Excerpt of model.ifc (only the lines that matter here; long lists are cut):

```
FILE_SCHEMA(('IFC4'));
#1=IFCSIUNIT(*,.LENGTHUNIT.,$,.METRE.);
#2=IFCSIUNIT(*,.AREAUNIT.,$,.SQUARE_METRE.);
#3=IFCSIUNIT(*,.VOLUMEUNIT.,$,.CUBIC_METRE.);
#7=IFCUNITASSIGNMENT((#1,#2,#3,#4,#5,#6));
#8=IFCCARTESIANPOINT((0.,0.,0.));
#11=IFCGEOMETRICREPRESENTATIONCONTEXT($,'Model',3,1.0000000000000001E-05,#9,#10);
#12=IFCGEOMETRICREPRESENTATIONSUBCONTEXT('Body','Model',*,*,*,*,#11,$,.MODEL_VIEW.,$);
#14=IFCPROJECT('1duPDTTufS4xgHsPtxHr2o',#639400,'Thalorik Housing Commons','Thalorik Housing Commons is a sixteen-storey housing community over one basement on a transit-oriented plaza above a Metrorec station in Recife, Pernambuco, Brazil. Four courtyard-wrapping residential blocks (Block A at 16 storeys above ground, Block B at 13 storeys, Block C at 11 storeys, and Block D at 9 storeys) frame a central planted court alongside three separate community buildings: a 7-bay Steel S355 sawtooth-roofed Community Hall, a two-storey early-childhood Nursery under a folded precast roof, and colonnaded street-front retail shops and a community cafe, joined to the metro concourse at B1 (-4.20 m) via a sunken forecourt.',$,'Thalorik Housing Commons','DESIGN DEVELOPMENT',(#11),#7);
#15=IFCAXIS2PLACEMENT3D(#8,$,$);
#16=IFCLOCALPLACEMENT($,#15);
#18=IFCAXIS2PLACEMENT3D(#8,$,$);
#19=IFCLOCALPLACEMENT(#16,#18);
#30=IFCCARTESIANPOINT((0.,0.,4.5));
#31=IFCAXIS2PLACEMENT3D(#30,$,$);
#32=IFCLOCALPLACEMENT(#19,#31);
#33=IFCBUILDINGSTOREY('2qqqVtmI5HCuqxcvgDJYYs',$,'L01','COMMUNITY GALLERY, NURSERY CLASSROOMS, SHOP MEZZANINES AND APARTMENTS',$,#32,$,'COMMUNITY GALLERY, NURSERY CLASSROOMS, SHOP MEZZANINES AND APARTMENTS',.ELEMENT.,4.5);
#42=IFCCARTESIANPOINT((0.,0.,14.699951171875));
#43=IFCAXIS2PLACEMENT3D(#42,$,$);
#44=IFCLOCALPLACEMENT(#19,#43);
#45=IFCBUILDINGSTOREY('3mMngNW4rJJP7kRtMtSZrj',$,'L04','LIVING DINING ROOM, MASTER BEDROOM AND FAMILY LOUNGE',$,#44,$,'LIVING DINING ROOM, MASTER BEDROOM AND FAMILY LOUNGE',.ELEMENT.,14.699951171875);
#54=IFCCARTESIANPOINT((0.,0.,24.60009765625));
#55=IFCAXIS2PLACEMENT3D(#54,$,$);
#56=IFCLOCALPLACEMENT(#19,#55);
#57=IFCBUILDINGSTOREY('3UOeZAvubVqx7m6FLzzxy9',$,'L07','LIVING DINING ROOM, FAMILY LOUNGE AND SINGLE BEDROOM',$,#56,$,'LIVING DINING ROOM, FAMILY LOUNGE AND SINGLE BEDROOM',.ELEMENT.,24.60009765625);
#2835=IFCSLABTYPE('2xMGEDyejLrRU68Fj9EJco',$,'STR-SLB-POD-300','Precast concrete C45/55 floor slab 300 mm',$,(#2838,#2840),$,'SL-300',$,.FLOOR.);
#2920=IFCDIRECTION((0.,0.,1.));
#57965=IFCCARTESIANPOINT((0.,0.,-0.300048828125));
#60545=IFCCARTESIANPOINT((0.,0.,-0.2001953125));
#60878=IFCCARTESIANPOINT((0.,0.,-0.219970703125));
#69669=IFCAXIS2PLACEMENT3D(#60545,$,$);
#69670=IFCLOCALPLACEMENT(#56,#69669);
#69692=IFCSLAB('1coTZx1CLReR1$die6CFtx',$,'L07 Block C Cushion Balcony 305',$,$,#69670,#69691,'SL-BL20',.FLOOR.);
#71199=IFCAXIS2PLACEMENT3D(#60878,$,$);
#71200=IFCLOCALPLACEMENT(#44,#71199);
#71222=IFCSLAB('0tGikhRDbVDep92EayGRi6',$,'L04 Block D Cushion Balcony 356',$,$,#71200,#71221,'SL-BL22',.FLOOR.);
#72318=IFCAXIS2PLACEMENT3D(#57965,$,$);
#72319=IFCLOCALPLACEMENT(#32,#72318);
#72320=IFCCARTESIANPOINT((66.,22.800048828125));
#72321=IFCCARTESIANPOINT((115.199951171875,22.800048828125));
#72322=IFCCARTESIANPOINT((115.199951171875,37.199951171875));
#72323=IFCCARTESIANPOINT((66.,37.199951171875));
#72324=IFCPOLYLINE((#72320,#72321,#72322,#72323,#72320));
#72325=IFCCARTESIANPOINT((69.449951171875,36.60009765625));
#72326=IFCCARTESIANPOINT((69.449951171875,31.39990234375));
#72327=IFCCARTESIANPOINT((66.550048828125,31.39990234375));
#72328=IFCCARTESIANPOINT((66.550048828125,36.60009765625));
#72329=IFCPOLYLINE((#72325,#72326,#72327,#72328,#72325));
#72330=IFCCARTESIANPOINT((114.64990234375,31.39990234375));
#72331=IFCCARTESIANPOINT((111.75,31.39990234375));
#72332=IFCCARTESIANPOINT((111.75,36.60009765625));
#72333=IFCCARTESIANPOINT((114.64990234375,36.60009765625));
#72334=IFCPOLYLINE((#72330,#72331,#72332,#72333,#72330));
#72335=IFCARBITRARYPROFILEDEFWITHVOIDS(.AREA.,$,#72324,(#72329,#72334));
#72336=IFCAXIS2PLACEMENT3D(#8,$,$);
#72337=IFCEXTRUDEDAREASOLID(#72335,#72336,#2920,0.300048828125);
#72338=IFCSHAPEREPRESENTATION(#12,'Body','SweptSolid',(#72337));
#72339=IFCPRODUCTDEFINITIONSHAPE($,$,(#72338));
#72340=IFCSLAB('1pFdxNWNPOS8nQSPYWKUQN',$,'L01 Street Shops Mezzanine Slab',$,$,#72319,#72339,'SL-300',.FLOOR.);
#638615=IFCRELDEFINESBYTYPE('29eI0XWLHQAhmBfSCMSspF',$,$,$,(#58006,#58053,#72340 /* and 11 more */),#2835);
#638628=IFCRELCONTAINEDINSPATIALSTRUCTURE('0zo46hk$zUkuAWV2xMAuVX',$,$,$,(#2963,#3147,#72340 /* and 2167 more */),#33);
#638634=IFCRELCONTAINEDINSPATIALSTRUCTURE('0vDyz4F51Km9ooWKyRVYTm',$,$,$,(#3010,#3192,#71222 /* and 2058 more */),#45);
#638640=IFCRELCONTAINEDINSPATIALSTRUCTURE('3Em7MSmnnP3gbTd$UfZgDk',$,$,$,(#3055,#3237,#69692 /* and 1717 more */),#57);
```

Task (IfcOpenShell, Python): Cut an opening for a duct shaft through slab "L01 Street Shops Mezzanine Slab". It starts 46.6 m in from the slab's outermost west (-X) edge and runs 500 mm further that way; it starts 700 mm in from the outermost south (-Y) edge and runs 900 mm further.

```python
import numpy as np
import ifcopenshell
import ifcopenshell.api.feature
import ifcopenshell.api.geometry
import ifcopenshell.api.root
import ifcopenshell.geom
import ifcopenshell.util.placement
import ifcopenshell.util.representation
import ifcopenshell.util.shape
import ifcopenshell.util.unit

model = ifcopenshell.open("model.ifc")
unit_scale = ifcopenshell.util.unit.calculate_unit_scale(model)
settings = ifcopenshell.geom.settings()


def volume(element):
    """Net volume in cubic metres, openings subtracted."""
    shape = ifcopenshell.geom.create_shape(settings, element)
    return ifcopenshell.util.shape.get_volume(shape.geometry)


slab = model.by_guid("1pFdxNWNPOS8nQSPYWKUQN")
before = volume(slab)

# Extent in the slab's own axes, in metres. The edges named are its -X and -Y sides.
slab_shape = ifcopenshell.geom.create_shape(settings, slab)
vertices = ifcopenshell.util.shape.get_vertices(slab_shape.geometry)
x_min, y_min, bottom = vertices.min(axis=0)
top = vertices[:, 2].max()

opening = ifcopenshell.api.root.create_entity(model, ifc_class="IfcOpeningElement", name="Duct shaft opening", predefined_type="OPENING")
context = ifcopenshell.util.representation.get_context(model, "Model", "Body", "MODEL_VIEW")
width, depth = 0.5, 0.9
outline = [(0.0, 0.0), (width, 0.0), (width, depth), (0.0, depth), (0.0, 0.0)]
# Overshoot both faces by 50 mm so the cut is clean.
shape = ifcopenshell.api.geometry.add_slab_representation(
    model, context=context, depth=top - bottom + 0.1, polyline=outline
)
ifcopenshell.api.geometry.assign_representation(model, product=opening, representation=shape)

matrix = ifcopenshell.util.placement.get_local_placement(slab.ObjectPlacement)
matrix[:, 3] = matrix @ np.append(np.array([x_min + 46.6, y_min + 0.7, bottom - 0.05]) / unit_scale, 1.0)
ifcopenshell.api.geometry.edit_object_placement(model, product=opening, matrix=matrix, is_si=False)
ifcopenshell.api.feature.add_feature(model, feature=opening, element=slab)

after = volume(slab)

print(f"slab volume {before:.3f} -> {after:.3f} m3")

model.write("model_edited.ifc")
```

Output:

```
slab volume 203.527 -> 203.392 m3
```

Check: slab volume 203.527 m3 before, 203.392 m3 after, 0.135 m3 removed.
